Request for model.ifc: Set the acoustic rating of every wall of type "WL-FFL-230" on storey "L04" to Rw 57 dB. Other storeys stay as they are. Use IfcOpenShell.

First a look at what the model holds.

```python
import ifcopenshell
import ifcopenshell.util.element

model = ifcopenshell.open("model.ifc")
print(model.schema)
storey = next(s for s in model.by_type("IfcBuildingStorey") if s.Name == "L04")
walls = [e for e in ifcopenshell.util.element.get_decomposition(storey) if e.is_a("IfcWall")]
seen = {}
for e in walls:
    element_type = ifcopenshell.util.element.get_type(e)
    key = (element_type.Name if element_type != e and element_type else None, ifcopenshell.util.element.get_pset(e, "Pset_WallCommon", "AcousticRating"))
    seen[key] = seen.get(key, 0) + 1
for (name, value), count in sorted(seen.items(), key=str):
    print(count, "x", name, "|", value)
```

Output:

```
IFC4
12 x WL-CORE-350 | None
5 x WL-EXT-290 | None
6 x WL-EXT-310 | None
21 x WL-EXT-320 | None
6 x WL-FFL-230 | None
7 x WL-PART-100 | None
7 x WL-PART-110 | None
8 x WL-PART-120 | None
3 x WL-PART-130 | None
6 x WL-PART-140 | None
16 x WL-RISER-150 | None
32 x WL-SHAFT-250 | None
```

```python
import ifcopenshell
import ifcopenshell.api.pset
import ifcopenshell.util.element

model = ifcopenshell.open("model.ifc")

storey = next(s for s in model.by_type("IfcBuildingStorey") if s.Name == "L04")
walls = [e for e in ifcopenshell.util.element.get_decomposition(storey) if e.is_a("IfcWall")]

count = 0
for e in walls:
    element_type = ifcopenshell.util.element.get_type(e)
    if element_type in (None, e) or element_type.Name != "WL-FFL-230":
        continue
    # add_pset returns the element's existing set when there is one.
    pset = ifcopenshell.api.pset.add_pset(model, product=e, name="Pset_WallCommon")
    ifcopenshell.api.pset.edit_pset(model, pset=pset, properties={"AcousticRating": "Rw 57 dB"})
    count += 1

print(count, "walls updated")

model.write("model_rev.ifc")
```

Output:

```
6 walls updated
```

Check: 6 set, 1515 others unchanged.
